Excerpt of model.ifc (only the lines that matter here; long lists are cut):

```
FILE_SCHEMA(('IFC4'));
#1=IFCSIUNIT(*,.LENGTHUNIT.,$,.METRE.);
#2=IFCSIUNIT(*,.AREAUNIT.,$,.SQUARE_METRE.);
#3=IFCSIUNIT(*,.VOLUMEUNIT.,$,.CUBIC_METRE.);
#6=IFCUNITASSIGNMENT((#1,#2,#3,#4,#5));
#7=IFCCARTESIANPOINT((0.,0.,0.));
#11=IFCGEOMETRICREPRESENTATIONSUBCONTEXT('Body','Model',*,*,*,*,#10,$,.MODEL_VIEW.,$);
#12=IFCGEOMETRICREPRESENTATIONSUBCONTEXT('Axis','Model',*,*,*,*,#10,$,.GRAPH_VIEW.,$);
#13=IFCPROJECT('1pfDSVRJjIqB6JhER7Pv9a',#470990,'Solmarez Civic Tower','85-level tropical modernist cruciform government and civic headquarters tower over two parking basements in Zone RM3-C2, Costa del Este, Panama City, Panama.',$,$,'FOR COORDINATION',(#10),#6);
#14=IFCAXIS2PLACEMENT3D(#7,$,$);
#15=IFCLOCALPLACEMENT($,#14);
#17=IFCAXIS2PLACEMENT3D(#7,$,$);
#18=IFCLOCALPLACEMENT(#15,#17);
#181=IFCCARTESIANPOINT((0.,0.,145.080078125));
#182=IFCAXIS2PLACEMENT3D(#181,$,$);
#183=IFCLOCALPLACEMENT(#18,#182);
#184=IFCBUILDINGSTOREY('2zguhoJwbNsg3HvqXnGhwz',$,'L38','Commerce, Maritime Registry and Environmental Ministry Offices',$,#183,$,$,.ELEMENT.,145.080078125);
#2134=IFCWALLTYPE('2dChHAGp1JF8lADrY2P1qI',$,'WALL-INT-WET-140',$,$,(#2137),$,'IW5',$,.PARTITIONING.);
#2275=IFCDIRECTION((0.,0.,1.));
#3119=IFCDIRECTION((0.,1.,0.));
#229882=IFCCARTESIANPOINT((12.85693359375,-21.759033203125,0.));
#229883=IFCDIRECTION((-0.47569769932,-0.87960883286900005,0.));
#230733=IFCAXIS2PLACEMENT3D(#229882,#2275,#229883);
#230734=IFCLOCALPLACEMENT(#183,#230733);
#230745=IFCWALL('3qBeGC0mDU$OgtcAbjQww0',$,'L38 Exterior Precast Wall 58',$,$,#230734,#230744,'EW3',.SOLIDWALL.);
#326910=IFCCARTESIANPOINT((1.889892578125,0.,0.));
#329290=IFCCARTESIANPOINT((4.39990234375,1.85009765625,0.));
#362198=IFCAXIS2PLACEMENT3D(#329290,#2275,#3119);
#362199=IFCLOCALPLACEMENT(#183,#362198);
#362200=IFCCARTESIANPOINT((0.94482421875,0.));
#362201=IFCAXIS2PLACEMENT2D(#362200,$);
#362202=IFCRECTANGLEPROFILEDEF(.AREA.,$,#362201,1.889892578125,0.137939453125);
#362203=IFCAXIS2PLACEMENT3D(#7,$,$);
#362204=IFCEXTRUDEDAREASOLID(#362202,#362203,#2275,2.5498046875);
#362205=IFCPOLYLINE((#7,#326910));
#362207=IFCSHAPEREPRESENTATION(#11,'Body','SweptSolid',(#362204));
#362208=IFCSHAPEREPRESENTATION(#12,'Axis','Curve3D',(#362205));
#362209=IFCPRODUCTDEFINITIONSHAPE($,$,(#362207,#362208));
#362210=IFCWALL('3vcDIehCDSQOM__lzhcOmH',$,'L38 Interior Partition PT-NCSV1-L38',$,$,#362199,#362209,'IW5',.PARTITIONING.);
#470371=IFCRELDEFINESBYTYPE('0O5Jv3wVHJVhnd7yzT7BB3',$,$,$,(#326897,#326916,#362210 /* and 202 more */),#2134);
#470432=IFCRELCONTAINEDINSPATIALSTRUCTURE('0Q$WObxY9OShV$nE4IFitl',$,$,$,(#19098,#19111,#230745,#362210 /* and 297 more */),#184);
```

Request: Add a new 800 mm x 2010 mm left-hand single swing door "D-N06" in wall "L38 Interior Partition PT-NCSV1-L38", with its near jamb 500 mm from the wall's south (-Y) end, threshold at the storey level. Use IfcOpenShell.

```python
import numpy as np
import ifcopenshell
import ifcopenshell.api.feature
import ifcopenshell.api.geometry
import ifcopenshell.api.root
import ifcopenshell.api.spatial
import ifcopenshell.geom
import ifcopenshell.util.element
import ifcopenshell.util.placement
import ifcopenshell.util.representation
import ifcopenshell.util.shape
import ifcopenshell.util.unit

model = ifcopenshell.open("model.ifc")
unit_scale = ifcopenshell.util.unit.calculate_unit_scale(model)
settings = ifcopenshell.geom.settings()


def volume(element):
    """Net volume in cubic metres, openings subtracted."""
    shape = ifcopenshell.geom.create_shape(settings, element)
    return ifcopenshell.util.shape.get_volume(shape.geometry)


wall = model.by_guid("3vcDIehCDSQOM__lzhcOmH")
storey = ifcopenshell.util.element.get_container(wall, ifc_class="IfcBuildingStorey")
context = ifcopenshell.util.representation.get_context(model, "Model", "Body", "MODEL_VIEW")
before = volume(wall)

width, height, from_end, sill = 0.8, 2.01, 0.5, 0.0  # metres

# The wall runs along its own X axis, and the end named is its -X end.
wall_shape = ifcopenshell.geom.create_shape(settings, wall)
x, y, z = ifcopenshell.util.shape.get_vertices(wall_shape.geometry).T
start = x.min() + from_end
face, thickness = float(y.min()), float(y.max() - y.min())
wall_matrix = ifcopenshell.util.placement.get_local_placement(wall.ObjectPlacement)
level = ifcopenshell.util.placement.get_local_placement(storey.ObjectPlacement)[2, 3]


def in_wall(x, y):
    """Placement at x, y metres in the wall's axes, at sill height."""
    matrix = wall_matrix.copy()
    matrix[:, 3] = wall_matrix @ np.array([x / unit_scale, y / unit_scale, 0.0, 1.0])
    matrix[2, 3] = level + sill / unit_scale
    return matrix


# Opening: a box that overshoots both wall faces by 50 mm.
opening = ifcopenshell.api.root.create_entity(model, ifc_class="IfcOpeningElement", predefined_type="OPENING")
box = ifcopenshell.api.geometry.add_wall_representation(
    model, context=context, length=width, height=height, thickness=thickness + 0.1
)
ifcopenshell.api.geometry.assign_representation(model, product=opening, representation=box)
ifcopenshell.api.geometry.edit_object_placement(model, product=opening, matrix=in_wall(start, face - 0.05), is_si=False)
ifcopenshell.api.feature.add_feature(model, feature=opening, element=wall)

door = ifcopenshell.api.root.create_entity(model, ifc_class="IfcDoor", name="D-N06", predefined_type="DOOR")
door.OverallWidth, door.OverallHeight = width / unit_scale, height / unit_scale
door.OperationType = "SINGLE_SWING_LEFT"
body = ifcopenshell.api.geometry.add_door_representation(
    model,
    context=context,
    overall_width=door.OverallWidth,
    overall_height=door.OverallHeight,
    operation_type="SINGLE_SWING_LEFT",
    lining_properties={"LiningDepth": thickness / unit_scale, "ThresholdDepth": thickness / unit_scale},
)
ifcopenshell.api.geometry.assign_representation(model, product=door, representation=body)
ifcopenshell.api.spatial.assign_container(model, products=[door], relating_structure=storey)
ifcopenshell.api.feature.add_filling(model, opening=opening, element=door)

# The lining spans the wall, so the door starts at the wall face.
ifcopenshell.api.geometry.edit_object_placement(model, product=door, matrix=in_wall(start, face), is_si=False)

after = volume(wall)

print(f"wall volume {before:.3f} -> {after:.3f} m3")

model.write("model-out.ifc")
```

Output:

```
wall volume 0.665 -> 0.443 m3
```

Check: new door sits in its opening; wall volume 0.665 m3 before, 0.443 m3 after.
